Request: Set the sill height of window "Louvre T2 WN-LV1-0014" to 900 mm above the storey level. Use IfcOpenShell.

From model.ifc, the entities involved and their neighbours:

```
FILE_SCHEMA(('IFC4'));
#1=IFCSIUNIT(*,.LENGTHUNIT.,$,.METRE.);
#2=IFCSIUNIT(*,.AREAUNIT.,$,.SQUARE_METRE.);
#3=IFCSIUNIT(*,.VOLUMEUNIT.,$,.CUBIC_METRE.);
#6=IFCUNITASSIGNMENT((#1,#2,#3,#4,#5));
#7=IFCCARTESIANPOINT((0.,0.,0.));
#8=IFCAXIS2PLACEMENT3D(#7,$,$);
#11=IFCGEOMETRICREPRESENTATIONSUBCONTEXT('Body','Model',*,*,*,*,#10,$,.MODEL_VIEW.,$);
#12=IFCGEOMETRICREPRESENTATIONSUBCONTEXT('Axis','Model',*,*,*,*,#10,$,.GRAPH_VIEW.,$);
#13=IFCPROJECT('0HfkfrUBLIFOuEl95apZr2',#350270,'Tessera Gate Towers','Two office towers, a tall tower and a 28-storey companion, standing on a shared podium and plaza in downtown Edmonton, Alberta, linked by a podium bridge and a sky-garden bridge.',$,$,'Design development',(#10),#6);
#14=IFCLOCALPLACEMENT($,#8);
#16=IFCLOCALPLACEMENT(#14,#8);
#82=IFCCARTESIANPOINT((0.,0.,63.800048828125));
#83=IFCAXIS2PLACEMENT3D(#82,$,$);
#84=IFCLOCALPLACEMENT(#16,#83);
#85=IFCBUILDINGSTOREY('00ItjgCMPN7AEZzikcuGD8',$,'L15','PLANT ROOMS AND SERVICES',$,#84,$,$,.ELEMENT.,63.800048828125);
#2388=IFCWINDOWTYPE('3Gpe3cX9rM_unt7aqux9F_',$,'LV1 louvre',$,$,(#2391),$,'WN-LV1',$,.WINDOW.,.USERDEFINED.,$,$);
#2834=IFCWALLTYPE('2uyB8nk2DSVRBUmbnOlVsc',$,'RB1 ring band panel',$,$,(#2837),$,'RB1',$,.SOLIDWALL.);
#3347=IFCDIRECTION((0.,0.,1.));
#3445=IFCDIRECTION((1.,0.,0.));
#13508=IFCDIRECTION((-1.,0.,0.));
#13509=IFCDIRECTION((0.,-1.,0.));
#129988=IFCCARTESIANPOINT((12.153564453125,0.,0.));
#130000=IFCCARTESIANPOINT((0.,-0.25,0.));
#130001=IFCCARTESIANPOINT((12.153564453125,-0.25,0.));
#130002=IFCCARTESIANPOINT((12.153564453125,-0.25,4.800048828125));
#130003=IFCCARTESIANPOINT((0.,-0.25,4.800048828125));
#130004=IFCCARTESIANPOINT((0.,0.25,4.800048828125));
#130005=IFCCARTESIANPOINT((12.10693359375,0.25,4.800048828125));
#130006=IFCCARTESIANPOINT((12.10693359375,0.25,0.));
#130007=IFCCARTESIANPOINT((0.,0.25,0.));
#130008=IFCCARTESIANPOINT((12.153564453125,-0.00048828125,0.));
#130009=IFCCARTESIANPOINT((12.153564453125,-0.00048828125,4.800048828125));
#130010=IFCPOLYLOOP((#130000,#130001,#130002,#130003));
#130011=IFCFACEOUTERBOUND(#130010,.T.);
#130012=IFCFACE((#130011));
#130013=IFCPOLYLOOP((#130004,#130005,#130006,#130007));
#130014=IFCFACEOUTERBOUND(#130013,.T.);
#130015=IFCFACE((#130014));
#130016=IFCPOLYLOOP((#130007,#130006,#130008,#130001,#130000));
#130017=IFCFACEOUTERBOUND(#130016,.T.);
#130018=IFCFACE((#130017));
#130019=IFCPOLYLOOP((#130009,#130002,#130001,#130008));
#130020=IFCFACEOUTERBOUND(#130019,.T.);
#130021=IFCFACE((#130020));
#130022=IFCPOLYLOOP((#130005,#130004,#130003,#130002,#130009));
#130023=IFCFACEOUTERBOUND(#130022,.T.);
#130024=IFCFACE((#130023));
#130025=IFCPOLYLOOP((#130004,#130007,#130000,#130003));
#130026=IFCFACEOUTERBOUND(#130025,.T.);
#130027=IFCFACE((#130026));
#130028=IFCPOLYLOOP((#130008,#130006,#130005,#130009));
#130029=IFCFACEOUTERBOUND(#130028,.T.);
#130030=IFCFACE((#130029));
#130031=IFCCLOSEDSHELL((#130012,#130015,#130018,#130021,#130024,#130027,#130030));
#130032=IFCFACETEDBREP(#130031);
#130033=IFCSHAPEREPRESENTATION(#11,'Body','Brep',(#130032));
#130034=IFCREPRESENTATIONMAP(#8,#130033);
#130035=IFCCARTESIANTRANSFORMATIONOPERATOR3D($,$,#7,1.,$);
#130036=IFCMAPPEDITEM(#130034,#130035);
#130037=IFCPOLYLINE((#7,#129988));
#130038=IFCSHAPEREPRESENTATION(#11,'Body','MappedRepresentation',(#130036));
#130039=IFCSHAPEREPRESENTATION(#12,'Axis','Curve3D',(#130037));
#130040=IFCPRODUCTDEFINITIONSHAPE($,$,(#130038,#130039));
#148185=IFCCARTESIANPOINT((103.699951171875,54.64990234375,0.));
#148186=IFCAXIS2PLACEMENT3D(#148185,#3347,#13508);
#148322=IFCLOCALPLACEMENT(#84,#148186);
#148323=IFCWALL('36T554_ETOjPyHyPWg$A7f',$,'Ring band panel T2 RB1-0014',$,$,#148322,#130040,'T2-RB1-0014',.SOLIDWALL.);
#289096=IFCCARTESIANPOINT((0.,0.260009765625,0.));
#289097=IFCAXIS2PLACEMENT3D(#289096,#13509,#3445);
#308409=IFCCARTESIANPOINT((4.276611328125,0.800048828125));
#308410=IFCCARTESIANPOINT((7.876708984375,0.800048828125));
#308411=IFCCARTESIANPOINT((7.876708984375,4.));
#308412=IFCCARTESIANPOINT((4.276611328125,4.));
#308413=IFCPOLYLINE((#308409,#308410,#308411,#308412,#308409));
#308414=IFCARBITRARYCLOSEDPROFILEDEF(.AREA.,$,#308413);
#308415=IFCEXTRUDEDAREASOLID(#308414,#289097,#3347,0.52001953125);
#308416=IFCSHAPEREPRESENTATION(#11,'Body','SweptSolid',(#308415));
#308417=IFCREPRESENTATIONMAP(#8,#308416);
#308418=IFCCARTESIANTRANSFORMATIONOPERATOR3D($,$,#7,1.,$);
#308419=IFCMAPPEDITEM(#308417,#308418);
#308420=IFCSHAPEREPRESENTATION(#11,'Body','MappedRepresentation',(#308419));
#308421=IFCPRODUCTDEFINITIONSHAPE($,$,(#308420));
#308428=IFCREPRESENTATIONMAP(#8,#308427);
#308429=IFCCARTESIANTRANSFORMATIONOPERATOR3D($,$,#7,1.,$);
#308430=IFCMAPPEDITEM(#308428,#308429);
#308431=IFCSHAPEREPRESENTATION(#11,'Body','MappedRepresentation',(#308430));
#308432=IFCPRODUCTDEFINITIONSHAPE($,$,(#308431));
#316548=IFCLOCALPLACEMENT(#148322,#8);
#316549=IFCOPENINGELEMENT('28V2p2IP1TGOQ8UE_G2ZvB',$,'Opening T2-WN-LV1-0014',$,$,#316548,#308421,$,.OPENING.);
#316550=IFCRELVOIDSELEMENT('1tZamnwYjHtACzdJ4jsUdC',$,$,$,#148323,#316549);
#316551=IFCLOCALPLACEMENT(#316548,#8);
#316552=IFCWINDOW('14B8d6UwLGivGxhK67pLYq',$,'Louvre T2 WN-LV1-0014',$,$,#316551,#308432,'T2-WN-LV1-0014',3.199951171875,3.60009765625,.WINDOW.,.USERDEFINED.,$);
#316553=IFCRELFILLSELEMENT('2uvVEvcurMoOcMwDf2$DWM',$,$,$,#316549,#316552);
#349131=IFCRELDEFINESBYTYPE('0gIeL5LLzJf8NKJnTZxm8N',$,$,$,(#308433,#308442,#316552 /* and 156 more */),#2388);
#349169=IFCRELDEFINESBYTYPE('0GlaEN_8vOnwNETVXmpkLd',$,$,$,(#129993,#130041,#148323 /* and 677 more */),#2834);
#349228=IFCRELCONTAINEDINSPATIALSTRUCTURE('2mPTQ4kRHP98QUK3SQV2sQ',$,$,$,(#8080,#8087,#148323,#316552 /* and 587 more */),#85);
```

```python
import numpy as np
import ifcopenshell
import ifcopenshell.api.geometry
import ifcopenshell.geom
import ifcopenshell.util.element
import ifcopenshell.util.placement
import ifcopenshell.util.shape
import ifcopenshell.util.unit

model = ifcopenshell.open("model.ifc")
unit_scale = ifcopenshell.util.unit.calculate_unit_scale(model)

window = model.by_guid("14B8d6UwLGivGxhK67pLYq")
opening = window.FillsVoids[0].RelatingOpeningElement
storey = ifcopenshell.util.element.get_container(window, ifc_class="IfcBuildingStorey")
level = ifcopenshell.util.placement.get_local_placement(storey.ObjectPlacement)[2, 3]

# The opening's origin need not be at the sill, so measure its lowest point.
shape = ifcopenshell.geom.create_shape(ifcopenshell.geom.settings(), opening)
bottom = ifcopenshell.util.shape.get_shape_bottom_elevation(shape, shape.geometry) / unit_scale
dz = level + 0.9 - bottom

shift = np.array([0.0, 0.0, dz])
# The window is placed relative to its opening, so it follows when the opening moves.
matrix = ifcopenshell.util.placement.get_local_placement(opening.ObjectPlacement)
matrix[:3, 3] += shift
ifcopenshell.api.geometry.edit_object_placement(
    model, product=opening, matrix=matrix, is_si=False, should_transform_children=True
)

print(f"moved by {dz * unit_scale:+.3f} m")

model.write("model_v2.ifc")
```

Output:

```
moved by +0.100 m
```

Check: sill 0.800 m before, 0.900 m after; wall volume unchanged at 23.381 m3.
